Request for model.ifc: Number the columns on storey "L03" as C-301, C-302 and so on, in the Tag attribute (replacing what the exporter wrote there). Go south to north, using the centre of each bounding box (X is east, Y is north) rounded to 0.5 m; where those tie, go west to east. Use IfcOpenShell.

First a look at what the model holds.

```python
import ifcopenshell
import ifcopenshell.util.element
import ifcopenshell.util.placement

model = ifcopenshell.open("model.ifc")
print(model.schema)
storey = next(s for s in model.by_type("IfcBuildingStorey") if s.Name == "L03")
columns = [e for e in ifcopenshell.util.element.get_decomposition(storey) if e.is_a("IfcColumn")]
for e in sorted(columns, key=lambda e: e.id()):
    origin = ifcopenshell.util.placement.get_local_placement(e.ObjectPlacement)[:3, 3]
    print(e.id(), e.Tag, e.Name, origin.round(2) + 0.0, sep=" | ")
```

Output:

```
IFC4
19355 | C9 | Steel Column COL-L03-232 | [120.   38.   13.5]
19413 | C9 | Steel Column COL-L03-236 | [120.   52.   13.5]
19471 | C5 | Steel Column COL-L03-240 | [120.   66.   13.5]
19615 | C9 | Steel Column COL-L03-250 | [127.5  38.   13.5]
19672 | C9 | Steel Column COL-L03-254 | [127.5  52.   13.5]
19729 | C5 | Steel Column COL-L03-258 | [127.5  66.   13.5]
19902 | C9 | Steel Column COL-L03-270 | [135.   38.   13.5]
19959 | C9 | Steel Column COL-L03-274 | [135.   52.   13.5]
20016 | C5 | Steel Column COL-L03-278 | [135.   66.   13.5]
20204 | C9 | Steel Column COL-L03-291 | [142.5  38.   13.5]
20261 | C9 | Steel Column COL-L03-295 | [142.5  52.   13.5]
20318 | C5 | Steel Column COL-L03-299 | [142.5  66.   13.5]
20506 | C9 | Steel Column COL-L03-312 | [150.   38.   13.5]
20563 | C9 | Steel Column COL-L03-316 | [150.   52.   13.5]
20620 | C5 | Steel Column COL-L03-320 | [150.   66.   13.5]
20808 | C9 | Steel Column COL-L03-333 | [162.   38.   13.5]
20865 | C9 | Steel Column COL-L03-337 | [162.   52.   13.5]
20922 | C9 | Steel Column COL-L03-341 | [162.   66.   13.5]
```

```python
import ifcopenshell
import ifcopenshell.geom
import ifcopenshell.util.element
import ifcopenshell.util.shape

model = ifcopenshell.open("model.ifc")
settings = ifcopenshell.geom.settings()
settings.set("use-world-coords", True)


def centre(element):
    shape = ifcopenshell.geom.create_shape(settings, element)
    return ifcopenshell.util.shape.get_bbox_centroid(shape.geometry)


storey = next(s for s in model.by_type("IfcBuildingStorey") if s.Name == "L03")
columns = [e for e in ifcopenshell.util.element.get_decomposition(storey) if e.is_a("IfcColumn")]

# Insertion points can sit at a corner or the storey origin, so sort by the geometry (in metres).
centres = {e: centre(e) for e in columns}
columns.sort(key=lambda e: (round(centres[e][1] / 0.5), centres[e][0]))

for i, e in enumerate(columns, start=1):
    number = f"C-3{i:02d}"
    e.Tag = number
    print(e.id(), number)

model.write("model-out.ifc")
```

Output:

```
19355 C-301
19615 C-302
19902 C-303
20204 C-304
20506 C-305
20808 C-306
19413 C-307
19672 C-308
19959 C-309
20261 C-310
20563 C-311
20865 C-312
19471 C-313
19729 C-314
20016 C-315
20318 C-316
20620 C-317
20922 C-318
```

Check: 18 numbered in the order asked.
